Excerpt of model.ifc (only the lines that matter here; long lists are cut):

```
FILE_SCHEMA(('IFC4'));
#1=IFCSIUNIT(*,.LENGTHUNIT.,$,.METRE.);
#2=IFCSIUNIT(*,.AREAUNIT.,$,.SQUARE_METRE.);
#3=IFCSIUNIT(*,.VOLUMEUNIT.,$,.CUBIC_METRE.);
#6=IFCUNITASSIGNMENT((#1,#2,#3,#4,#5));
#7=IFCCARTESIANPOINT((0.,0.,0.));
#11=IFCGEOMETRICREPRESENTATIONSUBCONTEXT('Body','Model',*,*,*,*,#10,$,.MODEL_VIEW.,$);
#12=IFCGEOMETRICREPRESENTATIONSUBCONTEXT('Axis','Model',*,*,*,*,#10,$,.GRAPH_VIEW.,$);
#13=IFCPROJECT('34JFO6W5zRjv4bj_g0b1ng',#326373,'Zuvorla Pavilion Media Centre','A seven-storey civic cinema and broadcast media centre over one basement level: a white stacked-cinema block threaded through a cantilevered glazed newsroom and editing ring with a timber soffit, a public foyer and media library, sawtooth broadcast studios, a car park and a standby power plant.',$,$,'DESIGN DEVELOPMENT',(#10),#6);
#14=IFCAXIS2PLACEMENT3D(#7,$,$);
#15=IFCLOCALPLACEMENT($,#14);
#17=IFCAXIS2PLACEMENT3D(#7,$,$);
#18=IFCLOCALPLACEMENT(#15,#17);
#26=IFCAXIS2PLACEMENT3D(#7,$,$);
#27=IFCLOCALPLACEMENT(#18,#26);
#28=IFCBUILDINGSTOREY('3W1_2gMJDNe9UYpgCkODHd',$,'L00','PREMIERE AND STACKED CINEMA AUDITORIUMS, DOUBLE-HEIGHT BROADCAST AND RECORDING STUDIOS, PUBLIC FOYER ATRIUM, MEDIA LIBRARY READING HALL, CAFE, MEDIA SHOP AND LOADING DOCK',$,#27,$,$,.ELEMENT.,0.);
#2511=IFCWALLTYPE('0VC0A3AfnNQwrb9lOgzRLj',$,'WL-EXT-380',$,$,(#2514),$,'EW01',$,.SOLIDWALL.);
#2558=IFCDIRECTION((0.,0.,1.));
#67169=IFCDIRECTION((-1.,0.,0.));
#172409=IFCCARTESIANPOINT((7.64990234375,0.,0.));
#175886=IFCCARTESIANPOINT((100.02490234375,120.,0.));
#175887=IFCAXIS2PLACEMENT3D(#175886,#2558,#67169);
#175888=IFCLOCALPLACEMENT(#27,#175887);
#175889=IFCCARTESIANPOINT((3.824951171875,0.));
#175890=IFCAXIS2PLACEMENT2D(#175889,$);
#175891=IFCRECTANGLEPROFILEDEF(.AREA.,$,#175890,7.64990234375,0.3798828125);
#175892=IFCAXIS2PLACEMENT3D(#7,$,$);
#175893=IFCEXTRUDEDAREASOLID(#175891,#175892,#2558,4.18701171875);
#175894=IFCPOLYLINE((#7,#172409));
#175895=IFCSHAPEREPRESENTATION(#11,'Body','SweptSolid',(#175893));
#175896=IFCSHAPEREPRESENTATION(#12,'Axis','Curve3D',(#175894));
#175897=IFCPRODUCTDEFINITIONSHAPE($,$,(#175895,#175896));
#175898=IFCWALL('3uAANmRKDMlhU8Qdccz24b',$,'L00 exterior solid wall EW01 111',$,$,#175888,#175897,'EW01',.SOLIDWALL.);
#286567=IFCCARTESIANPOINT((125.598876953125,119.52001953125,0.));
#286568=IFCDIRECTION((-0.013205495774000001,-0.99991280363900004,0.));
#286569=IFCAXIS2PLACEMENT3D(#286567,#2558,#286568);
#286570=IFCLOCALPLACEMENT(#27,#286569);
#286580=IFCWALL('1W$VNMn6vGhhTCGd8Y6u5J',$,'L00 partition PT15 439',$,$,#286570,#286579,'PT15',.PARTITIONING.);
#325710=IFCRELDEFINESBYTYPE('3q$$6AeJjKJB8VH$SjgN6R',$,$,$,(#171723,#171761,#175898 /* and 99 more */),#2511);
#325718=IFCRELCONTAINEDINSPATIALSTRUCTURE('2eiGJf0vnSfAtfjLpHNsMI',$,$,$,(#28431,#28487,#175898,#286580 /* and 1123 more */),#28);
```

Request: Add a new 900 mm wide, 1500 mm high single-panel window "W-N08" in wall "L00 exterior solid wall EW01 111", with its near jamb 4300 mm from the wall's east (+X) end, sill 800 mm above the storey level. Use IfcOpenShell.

```python
import numpy as np
import ifcopenshell
import ifcopenshell.api.feature
import ifcopenshell.api.geometry
import ifcopenshell.api.root
import ifcopenshell.api.spatial
import ifcopenshell.geom
import ifcopenshell.util.element
import ifcopenshell.util.placement
import ifcopenshell.util.representation
import ifcopenshell.util.shape
import ifcopenshell.util.unit

model = ifcopenshell.open("model.ifc")
unit_scale = ifcopenshell.util.unit.calculate_unit_scale(model)
settings = ifcopenshell.geom.settings()


def volume(element):
    """Net volume in cubic metres, openings subtracted."""
    shape = ifcopenshell.geom.create_shape(settings, element)
    return ifcopenshell.util.shape.get_volume(shape.geometry)


wall = model.by_guid("3uAANmRKDMlhU8Qdccz24b")
storey = ifcopenshell.util.element.get_container(wall, ifc_class="IfcBuildingStorey")
context = ifcopenshell.util.representation.get_context(model, "Model", "Body", "MODEL_VIEW")
before = volume(wall)

width, height, from_end, sill = 0.9, 1.5, 4.3, 0.8  # metres

# The wall runs along its own X axis, and the end named is its -X end.
wall_shape = ifcopenshell.geom.create_shape(settings, wall)
x, y, z = ifcopenshell.util.shape.get_vertices(wall_shape.geometry).T
start = x.min() + from_end
face, thickness = float(y.min()), float(y.max() - y.min())
wall_matrix = ifcopenshell.util.placement.get_local_placement(wall.ObjectPlacement)
level = ifcopenshell.util.placement.get_local_placement(storey.ObjectPlacement)[2, 3]


def in_wall(x, y):
    """Placement at x, y metres in the wall's axes, at sill height."""
    matrix = wall_matrix.copy()
    matrix[:, 3] = wall_matrix @ np.array([x / unit_scale, y / unit_scale, 0.0, 1.0])
    matrix[2, 3] = level + sill / unit_scale
    return matrix


# Opening: a box that overshoots both wall faces by 50 mm.
opening = ifcopenshell.api.root.create_entity(model, ifc_class="IfcOpeningElement", predefined_type="OPENING")
box = ifcopenshell.api.geometry.add_wall_representation(
    model, context=context, length=width, height=height, thickness=thickness + 0.1
)
ifcopenshell.api.geometry.assign_representation(model, product=opening, representation=box)
ifcopenshell.api.geometry.edit_object_placement(model, product=opening, matrix=in_wall(start, face - 0.05), is_si=False)
ifcopenshell.api.feature.add_feature(model, feature=opening, element=wall)

window = ifcopenshell.api.root.create_entity(model, ifc_class="IfcWindow", name="W-N08", predefined_type="WINDOW")
window.OverallWidth, window.OverallHeight = width / unit_scale, height / unit_scale
window.PartitioningType = "SINGLE_PANEL"
body = ifcopenshell.api.geometry.add_window_representation(
    model,
    context=context,
    overall_width=window.OverallWidth,
    overall_height=window.OverallHeight,
    partition_type="SINGLE_PANEL",
)
ifcopenshell.api.geometry.assign_representation(model, product=window, representation=body)
ifcopenshell.api.spatial.assign_container(model, products=[window], relating_structure=storey)
ifcopenshell.api.feature.add_filling(model, opening=opening, element=window)

# Centre the window in the wall's thickness.
ifcopenshell.api.geometry.edit_object_placement(model, product=window, matrix=in_wall(start, face), is_si=False)
window_shape = ifcopenshell.geom.create_shape(settings, window)
depth = ifcopenshell.util.shape.get_vertices(window_shape.geometry)[:, 1]
offset = face + thickness / 2 - (depth.min() + depth.max()) / 2
ifcopenshell.api.geometry.edit_object_placement(model, product=window, matrix=in_wall(start, offset), is_si=False)

after = volume(wall)

print(f"wall volume {before:.3f} -> {after:.3f} m3")

model.write("model_edited.ifc")
```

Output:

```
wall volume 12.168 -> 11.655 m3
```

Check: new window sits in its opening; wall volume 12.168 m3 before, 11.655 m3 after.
